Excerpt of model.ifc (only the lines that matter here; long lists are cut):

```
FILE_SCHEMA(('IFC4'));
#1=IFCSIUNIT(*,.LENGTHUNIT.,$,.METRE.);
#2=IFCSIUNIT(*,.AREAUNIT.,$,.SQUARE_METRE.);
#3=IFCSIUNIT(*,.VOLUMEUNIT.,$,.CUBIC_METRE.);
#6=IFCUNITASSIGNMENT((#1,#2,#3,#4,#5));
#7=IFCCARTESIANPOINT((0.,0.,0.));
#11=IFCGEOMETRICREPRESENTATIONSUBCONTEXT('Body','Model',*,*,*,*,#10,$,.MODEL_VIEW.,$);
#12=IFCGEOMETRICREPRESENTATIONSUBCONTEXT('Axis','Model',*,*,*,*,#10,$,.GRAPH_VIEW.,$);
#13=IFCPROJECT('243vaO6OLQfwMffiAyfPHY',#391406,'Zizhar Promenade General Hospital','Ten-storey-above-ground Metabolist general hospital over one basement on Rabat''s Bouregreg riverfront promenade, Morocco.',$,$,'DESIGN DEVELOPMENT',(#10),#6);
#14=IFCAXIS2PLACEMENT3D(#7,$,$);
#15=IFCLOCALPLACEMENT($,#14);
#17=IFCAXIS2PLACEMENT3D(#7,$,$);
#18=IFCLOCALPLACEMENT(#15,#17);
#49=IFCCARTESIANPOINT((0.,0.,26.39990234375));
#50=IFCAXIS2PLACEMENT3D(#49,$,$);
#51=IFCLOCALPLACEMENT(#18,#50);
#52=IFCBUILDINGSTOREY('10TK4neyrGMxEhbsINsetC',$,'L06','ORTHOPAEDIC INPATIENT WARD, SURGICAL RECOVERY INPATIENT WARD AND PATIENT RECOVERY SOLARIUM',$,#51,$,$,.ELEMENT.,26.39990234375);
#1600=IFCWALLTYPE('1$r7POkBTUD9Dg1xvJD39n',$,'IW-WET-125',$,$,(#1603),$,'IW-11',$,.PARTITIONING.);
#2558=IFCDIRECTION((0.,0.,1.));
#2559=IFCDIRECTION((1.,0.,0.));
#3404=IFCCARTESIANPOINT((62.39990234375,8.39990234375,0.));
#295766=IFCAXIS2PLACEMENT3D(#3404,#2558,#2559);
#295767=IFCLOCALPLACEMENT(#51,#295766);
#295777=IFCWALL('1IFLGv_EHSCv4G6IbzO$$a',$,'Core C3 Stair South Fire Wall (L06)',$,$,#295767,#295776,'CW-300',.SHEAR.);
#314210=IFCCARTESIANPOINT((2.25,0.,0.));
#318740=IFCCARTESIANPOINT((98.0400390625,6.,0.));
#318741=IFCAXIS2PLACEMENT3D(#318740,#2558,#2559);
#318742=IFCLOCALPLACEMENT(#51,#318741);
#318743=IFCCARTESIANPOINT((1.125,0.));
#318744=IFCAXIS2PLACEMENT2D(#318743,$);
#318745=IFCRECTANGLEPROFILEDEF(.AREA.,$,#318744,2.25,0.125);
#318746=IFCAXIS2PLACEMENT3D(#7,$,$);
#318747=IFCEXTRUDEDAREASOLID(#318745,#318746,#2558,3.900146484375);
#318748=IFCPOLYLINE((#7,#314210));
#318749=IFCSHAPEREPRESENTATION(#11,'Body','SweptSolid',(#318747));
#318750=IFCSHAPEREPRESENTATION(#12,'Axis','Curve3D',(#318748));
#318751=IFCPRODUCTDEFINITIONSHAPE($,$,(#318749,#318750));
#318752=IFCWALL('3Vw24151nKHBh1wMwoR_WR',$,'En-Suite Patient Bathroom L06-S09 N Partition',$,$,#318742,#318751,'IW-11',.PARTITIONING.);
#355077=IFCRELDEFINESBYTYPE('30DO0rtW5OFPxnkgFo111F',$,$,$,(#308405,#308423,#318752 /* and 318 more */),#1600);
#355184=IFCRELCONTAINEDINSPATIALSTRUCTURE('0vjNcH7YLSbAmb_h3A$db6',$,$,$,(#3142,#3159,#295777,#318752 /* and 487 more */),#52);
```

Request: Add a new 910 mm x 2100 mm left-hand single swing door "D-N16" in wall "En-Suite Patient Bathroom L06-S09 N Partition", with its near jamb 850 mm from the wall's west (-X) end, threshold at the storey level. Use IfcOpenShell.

```python
import numpy as np
import ifcopenshell
import ifcopenshell.api.feature
import ifcopenshell.api.geometry
import ifcopenshell.api.root
import ifcopenshell.api.spatial
import ifcopenshell.geom
import ifcopenshell.util.element
import ifcopenshell.util.placement
import ifcopenshell.util.representation
import ifcopenshell.util.shape
import ifcopenshell.util.unit

model = ifcopenshell.open("model.ifc")
unit_scale = ifcopenshell.util.unit.calculate_unit_scale(model)
settings = ifcopenshell.geom.settings()


def volume(element):
    """Net volume in cubic metres, openings subtracted."""
    shape = ifcopenshell.geom.create_shape(settings, element)
    return ifcopenshell.util.shape.get_volume(shape.geometry)


wall = model.by_id(318752)
storey = ifcopenshell.util.element.get_container(wall, ifc_class="IfcBuildingStorey")
context = ifcopenshell.util.representation.get_context(model, "Model", "Body", "MODEL_VIEW")
before = volume(wall)

width, height, from_end, sill = 0.91, 2.1, 0.85, 0.0  # metres

# The wall runs along its own X axis, and the end named is its -X end.
wall_shape = ifcopenshell.geom.create_shape(settings, wall)
x, y, z = ifcopenshell.util.shape.get_vertices(wall_shape.geometry).T
start = x.min() + from_end
face, thickness = float(y.min()), float(y.max() - y.min())
wall_matrix = ifcopenshell.util.placement.get_local_placement(wall.ObjectPlacement)
level = ifcopenshell.util.placement.get_local_placement(storey.ObjectPlacement)[2, 3]


def in_wall(x, y):
    """Placement at x, y metres in the wall's axes, at sill height."""
    matrix = wall_matrix.copy()
    matrix[:, 3] = wall_matrix @ np.array([x / unit_scale, y / unit_scale, 0.0, 1.0])
    matrix[2, 3] = level + sill / unit_scale
    return matrix


# Opening: a box that overshoots both wall faces by 50 mm.
opening = ifcopenshell.api.root.create_entity(model, ifc_class="IfcOpeningElement", predefined_type="OPENING")
box = ifcopenshell.api.geometry.add_wall_representation(
    model, context=context, length=width, height=height, thickness=thickness + 0.1
)
ifcopenshell.api.geometry.assign_representation(model, product=opening, representation=box)
ifcopenshell.api.geometry.edit_object_placement(model, product=opening, matrix=in_wall(start, face - 0.05), is_si=False)
ifcopenshell.api.feature.add_feature(model, feature=opening, element=wall)

door = ifcopenshell.api.root.create_entity(model, ifc_class="IfcDoor", name="D-N16", predefined_type="DOOR")
door.OverallWidth, door.OverallHeight = width / unit_scale, height / unit_scale
door.OperationType = "SINGLE_SWING_LEFT"
body = ifcopenshell.api.geometry.add_door_representation(
    model,
    context=context,
    overall_width=door.OverallWidth,
    overall_height=door.OverallHeight,
    operation_type="SINGLE_SWING_LEFT",
    lining_properties={"LiningDepth": thickness / unit_scale, "ThresholdDepth": thickness / unit_scale},
)
ifcopenshell.api.geometry.assign_representation(model, product=door, representation=body)
ifcopenshell.api.spatial.assign_container(model, products=[door], relating_structure=storey)
ifcopenshell.api.feature.add_filling(model, opening=opening, element=door)

# The lining spans the wall, so the door starts at the wall face.
ifcopenshell.api.geometry.edit_object_placement(model, product=door, matrix=in_wall(start, face), is_si=False)

after = volume(wall)

print(f"wall volume {before:.3f} -> {after:.3f} m3")

model.write("model_edited.ifc")
```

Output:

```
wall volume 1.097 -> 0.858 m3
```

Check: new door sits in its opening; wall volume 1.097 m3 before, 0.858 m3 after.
